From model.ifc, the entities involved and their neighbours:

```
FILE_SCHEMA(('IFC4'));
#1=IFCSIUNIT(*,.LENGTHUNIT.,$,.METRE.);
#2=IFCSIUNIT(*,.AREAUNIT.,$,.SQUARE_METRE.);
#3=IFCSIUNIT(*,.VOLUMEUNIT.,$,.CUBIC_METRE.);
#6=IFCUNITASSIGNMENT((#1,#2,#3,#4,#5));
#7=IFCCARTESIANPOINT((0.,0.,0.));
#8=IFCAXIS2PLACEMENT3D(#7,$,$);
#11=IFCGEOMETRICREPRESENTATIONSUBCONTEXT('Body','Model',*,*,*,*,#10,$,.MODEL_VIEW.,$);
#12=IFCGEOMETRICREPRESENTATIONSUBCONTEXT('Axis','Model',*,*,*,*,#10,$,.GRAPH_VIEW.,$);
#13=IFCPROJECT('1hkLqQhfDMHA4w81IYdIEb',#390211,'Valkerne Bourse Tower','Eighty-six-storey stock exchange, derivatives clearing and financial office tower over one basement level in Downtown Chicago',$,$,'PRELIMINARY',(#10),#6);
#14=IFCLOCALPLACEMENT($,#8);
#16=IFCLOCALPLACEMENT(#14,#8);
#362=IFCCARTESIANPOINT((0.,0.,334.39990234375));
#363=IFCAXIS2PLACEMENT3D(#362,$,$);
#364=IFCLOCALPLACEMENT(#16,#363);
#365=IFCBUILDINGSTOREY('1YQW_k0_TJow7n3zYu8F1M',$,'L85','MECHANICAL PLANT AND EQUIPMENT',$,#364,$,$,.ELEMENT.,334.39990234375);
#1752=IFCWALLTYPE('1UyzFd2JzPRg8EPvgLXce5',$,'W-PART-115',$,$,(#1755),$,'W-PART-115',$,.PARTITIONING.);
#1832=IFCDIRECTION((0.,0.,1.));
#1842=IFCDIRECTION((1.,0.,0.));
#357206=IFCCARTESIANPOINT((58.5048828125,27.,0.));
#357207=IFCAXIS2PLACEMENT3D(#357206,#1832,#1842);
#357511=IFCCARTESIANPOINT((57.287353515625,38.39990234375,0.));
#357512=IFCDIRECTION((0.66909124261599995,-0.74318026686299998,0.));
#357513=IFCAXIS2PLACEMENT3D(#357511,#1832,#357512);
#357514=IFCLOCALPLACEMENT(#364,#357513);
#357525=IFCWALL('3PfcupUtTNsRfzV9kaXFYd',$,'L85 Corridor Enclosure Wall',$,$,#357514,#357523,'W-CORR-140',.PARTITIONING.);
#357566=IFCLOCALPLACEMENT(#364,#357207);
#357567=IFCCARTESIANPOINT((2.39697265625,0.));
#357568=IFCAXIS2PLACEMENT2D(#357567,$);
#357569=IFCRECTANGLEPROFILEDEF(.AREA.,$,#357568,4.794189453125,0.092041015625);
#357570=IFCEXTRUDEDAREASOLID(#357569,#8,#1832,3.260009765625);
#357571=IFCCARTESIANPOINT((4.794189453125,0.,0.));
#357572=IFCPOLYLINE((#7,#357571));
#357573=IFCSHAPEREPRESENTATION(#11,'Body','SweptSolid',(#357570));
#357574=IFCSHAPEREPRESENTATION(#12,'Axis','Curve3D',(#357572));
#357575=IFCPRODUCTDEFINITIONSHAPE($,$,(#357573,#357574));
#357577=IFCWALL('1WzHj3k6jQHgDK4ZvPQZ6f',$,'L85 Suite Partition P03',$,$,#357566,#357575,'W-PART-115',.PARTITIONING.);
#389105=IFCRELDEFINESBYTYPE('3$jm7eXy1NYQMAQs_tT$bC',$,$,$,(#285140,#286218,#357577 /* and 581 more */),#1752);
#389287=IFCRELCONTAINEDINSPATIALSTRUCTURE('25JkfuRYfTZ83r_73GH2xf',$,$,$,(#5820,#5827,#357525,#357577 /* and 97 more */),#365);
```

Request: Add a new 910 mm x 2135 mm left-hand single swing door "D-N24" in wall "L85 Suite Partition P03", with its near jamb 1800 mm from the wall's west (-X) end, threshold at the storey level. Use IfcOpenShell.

```python
import numpy as np
import ifcopenshell
import ifcopenshell.api.feature
import ifcopenshell.api.geometry
import ifcopenshell.api.root
import ifcopenshell.api.spatial
import ifcopenshell.geom
import ifcopenshell.util.element
import ifcopenshell.util.placement
import ifcopenshell.util.representation
import ifcopenshell.util.shape
import ifcopenshell.util.unit

model = ifcopenshell.open("model.ifc")
unit_scale = ifcopenshell.util.unit.calculate_unit_scale(model)
settings = ifcopenshell.geom.settings()


def volume(element):
    """Net volume in cubic metres, openings subtracted."""
    shape = ifcopenshell.geom.create_shape(settings, element)
    return ifcopenshell.util.shape.get_volume(shape.geometry)


wall = model.by_guid("1WzHj3k6jQHgDK4ZvPQZ6f")
storey = ifcopenshell.util.element.get_container(wall, ifc_class="IfcBuildingStorey")
context = ifcopenshell.util.representation.get_context(model, "Model", "Body", "MODEL_VIEW")
before = volume(wall)

width, height, from_end, sill = 0.91, 2.135, 1.8, 0.0  # metres

# The wall runs along its own X axis, and the end named is its -X end.
wall_shape = ifcopenshell.geom.create_shape(settings, wall)
x, y, z = ifcopenshell.util.shape.get_vertices(wall_shape.geometry).T
start = x.min() + from_end
face, thickness = float(y.min()), float(y.max() - y.min())
wall_matrix = ifcopenshell.util.placement.get_local_placement(wall.ObjectPlacement)
level = ifcopenshell.util.placement.get_local_placement(storey.ObjectPlacement)[2, 3]


def in_wall(x, y):
    """Placement at x, y metres in the wall's axes, at sill height."""
    matrix = wall_matrix.copy()
    matrix[:, 3] = wall_matrix @ np.array([x / unit_scale, y / unit_scale, 0.0, 1.0])
    matrix[2, 3] = level + sill / unit_scale
    return matrix


# Opening: a box that overshoots both wall faces by 50 mm.
opening = ifcopenshell.api.root.create_entity(model, ifc_class="IfcOpeningElement", predefined_type="OPENING")
box = ifcopenshell.api.geometry.add_wall_representation(
    model, context=context, length=width, height=height, thickness=thickness + 0.1
)
ifcopenshell.api.geometry.assign_representation(model, product=opening, representation=box)
ifcopenshell.api.geometry.edit_object_placement(model, product=opening, matrix=in_wall(start, face - 0.05), is_si=False)
ifcopenshell.api.feature.add_feature(model, feature=opening, element=wall)

door = ifcopenshell.api.root.create_entity(model, ifc_class="IfcDoor", name="D-N24", predefined_type="DOOR")
door.OverallWidth, door.OverallHeight = width / unit_scale, height / unit_scale
door.OperationType = "SINGLE_SWING_LEFT"
body = ifcopenshell.api.geometry.add_door_representation(
    model,
    context=context,
    overall_width=door.OverallWidth,
    overall_height=door.OverallHeight,
    operation_type="SINGLE_SWING_LEFT",
    lining_properties={"LiningDepth": thickness / unit_scale, "ThresholdDepth": thickness / unit_scale},
)
ifcopenshell.api.geometry.assign_representation(model, product=door, representation=body)
ifcopenshell.api.spatial.assign_container(model, products=[door], relating_structure=storey)
ifcopenshell.api.feature.add_filling(model, opening=opening, element=door)

# The lining spans the wall, so the door starts at the wall face.
ifcopenshell.api.geometry.edit_object_placement(model, product=door, matrix=in_wall(start, face), is_si=False)

after = volume(wall)

print(f"wall volume {before:.3f} -> {after:.3f} m3")

model.write("model_edited.ifc")
```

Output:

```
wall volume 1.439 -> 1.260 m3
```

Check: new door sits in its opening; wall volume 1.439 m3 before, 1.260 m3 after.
